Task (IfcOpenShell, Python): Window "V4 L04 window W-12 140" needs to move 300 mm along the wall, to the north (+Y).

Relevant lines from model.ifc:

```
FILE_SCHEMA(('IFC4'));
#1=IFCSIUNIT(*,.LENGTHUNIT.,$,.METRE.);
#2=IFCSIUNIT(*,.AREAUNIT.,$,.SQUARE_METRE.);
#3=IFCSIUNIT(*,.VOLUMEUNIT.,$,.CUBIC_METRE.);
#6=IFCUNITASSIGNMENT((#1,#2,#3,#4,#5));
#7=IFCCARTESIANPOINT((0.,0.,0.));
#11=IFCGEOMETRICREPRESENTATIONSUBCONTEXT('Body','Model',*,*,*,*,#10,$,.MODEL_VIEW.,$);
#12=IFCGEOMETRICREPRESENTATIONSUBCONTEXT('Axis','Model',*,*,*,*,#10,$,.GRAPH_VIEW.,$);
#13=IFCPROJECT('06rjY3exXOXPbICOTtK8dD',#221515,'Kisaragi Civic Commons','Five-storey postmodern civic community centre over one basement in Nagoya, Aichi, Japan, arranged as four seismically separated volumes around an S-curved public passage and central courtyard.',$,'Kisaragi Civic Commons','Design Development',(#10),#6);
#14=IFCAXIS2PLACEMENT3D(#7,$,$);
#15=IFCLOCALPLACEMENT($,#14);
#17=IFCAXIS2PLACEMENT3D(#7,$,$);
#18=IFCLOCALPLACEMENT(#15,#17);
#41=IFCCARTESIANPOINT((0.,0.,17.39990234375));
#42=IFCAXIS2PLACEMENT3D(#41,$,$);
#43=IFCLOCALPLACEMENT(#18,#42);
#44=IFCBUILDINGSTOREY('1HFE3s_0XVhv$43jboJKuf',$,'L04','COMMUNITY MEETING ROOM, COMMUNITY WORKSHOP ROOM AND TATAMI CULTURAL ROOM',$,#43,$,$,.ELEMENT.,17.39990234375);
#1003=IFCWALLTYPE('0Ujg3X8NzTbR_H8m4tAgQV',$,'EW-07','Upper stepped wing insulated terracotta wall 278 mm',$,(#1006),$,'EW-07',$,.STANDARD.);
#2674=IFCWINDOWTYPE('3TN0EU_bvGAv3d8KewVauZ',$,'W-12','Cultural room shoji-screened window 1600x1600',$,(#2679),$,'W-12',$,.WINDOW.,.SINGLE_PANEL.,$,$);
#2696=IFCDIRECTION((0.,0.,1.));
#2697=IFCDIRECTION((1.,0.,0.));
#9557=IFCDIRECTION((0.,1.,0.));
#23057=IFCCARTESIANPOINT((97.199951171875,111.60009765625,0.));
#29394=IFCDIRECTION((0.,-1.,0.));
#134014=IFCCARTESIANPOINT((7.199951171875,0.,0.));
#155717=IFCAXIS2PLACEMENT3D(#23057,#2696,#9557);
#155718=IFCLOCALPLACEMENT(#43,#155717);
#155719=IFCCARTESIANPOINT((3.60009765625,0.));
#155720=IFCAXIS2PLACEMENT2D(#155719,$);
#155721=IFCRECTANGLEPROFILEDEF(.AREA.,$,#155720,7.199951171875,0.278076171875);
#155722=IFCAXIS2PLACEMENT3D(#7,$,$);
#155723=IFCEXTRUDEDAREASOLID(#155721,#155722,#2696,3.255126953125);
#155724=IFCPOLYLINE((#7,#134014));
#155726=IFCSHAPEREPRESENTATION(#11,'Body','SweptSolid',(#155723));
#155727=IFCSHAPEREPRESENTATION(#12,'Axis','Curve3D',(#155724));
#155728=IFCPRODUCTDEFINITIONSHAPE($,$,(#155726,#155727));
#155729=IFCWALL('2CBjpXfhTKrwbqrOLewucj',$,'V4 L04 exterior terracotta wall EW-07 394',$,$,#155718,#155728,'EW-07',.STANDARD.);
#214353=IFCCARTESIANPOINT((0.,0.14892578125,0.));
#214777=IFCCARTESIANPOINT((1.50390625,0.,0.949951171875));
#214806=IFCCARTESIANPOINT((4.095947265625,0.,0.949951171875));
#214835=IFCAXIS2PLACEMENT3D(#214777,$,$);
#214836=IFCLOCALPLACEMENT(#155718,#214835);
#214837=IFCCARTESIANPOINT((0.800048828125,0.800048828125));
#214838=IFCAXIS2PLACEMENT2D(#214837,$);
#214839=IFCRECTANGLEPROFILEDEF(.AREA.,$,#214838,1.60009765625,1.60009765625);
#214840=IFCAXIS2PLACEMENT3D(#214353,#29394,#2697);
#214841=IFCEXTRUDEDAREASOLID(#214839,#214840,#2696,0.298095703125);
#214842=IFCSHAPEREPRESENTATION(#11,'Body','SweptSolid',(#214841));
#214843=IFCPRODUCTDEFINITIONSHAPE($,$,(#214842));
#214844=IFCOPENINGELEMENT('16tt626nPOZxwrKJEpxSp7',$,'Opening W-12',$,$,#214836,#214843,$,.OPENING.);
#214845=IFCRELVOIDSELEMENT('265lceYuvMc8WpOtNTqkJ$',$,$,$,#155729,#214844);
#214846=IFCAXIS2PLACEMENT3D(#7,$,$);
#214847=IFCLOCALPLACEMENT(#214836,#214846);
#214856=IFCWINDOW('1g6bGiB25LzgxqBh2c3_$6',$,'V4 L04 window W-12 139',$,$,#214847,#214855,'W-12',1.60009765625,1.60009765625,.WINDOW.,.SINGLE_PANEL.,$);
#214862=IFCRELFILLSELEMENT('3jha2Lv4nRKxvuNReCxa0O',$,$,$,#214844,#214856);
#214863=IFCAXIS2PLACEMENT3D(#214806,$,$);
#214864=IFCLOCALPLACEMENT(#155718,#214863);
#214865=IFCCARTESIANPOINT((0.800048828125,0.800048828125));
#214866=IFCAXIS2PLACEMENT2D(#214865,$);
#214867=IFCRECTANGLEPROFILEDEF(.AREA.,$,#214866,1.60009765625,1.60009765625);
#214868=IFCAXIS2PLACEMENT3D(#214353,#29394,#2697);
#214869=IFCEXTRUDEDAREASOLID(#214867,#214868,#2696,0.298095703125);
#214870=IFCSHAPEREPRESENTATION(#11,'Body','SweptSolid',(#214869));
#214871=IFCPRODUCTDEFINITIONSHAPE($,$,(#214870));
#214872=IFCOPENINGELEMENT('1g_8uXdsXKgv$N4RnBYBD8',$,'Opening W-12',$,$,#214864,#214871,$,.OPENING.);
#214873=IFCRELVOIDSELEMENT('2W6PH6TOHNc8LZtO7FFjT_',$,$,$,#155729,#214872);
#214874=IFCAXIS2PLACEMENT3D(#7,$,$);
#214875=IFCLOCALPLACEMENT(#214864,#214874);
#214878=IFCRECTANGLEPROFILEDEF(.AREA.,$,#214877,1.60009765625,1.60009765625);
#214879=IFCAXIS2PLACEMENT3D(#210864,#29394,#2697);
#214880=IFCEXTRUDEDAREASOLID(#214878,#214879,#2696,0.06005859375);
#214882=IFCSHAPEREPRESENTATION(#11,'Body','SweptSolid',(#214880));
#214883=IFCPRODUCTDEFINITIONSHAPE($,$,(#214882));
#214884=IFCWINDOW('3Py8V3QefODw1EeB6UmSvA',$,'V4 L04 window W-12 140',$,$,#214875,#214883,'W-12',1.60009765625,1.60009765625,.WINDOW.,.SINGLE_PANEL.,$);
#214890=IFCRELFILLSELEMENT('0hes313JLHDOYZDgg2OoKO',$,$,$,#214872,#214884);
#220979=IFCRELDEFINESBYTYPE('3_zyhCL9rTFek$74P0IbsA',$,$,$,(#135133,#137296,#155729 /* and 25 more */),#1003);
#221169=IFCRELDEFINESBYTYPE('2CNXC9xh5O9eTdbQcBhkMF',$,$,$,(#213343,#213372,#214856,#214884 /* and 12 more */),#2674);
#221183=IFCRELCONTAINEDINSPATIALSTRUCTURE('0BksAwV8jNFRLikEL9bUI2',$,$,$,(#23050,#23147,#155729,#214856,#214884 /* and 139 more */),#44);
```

```python
import ifcopenshell
import ifcopenshell.api.geometry
import ifcopenshell.util.placement
import ifcopenshell.util.unit

model = ifcopenshell.open("model.ifc")
unit_scale = ifcopenshell.util.unit.calculate_unit_scale(model)

window = model.by_id(214884)
opening = window.FillsVoids[0].RelatingOpeningElement
wall = opening.VoidsElements[0].RelatingBuildingElement

wall_matrix = ifcopenshell.util.placement.get_local_placement(wall.ObjectPlacement)
shift = wall_matrix[:3, 0] * 0.3 / unit_scale
before = ifcopenshell.util.placement.get_local_placement(window.ObjectPlacement)[:3, 3].copy()

# The window is placed relative to its opening, so it follows when the opening moves.
matrix = ifcopenshell.util.placement.get_local_placement(opening.ObjectPlacement)
matrix[:3, 3] += shift
ifcopenshell.api.geometry.edit_object_placement(
    model, product=opening, matrix=matrix, is_si=False, should_transform_children=True
)

after = ifcopenshell.util.placement.get_local_placement(window.ObjectPlacement)[:3, 3]
print("window moved by", (after - before).round(3) + 0.0)

model.write("model-out.ifc")
```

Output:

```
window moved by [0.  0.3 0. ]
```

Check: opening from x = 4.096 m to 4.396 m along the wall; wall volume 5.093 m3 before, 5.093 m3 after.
